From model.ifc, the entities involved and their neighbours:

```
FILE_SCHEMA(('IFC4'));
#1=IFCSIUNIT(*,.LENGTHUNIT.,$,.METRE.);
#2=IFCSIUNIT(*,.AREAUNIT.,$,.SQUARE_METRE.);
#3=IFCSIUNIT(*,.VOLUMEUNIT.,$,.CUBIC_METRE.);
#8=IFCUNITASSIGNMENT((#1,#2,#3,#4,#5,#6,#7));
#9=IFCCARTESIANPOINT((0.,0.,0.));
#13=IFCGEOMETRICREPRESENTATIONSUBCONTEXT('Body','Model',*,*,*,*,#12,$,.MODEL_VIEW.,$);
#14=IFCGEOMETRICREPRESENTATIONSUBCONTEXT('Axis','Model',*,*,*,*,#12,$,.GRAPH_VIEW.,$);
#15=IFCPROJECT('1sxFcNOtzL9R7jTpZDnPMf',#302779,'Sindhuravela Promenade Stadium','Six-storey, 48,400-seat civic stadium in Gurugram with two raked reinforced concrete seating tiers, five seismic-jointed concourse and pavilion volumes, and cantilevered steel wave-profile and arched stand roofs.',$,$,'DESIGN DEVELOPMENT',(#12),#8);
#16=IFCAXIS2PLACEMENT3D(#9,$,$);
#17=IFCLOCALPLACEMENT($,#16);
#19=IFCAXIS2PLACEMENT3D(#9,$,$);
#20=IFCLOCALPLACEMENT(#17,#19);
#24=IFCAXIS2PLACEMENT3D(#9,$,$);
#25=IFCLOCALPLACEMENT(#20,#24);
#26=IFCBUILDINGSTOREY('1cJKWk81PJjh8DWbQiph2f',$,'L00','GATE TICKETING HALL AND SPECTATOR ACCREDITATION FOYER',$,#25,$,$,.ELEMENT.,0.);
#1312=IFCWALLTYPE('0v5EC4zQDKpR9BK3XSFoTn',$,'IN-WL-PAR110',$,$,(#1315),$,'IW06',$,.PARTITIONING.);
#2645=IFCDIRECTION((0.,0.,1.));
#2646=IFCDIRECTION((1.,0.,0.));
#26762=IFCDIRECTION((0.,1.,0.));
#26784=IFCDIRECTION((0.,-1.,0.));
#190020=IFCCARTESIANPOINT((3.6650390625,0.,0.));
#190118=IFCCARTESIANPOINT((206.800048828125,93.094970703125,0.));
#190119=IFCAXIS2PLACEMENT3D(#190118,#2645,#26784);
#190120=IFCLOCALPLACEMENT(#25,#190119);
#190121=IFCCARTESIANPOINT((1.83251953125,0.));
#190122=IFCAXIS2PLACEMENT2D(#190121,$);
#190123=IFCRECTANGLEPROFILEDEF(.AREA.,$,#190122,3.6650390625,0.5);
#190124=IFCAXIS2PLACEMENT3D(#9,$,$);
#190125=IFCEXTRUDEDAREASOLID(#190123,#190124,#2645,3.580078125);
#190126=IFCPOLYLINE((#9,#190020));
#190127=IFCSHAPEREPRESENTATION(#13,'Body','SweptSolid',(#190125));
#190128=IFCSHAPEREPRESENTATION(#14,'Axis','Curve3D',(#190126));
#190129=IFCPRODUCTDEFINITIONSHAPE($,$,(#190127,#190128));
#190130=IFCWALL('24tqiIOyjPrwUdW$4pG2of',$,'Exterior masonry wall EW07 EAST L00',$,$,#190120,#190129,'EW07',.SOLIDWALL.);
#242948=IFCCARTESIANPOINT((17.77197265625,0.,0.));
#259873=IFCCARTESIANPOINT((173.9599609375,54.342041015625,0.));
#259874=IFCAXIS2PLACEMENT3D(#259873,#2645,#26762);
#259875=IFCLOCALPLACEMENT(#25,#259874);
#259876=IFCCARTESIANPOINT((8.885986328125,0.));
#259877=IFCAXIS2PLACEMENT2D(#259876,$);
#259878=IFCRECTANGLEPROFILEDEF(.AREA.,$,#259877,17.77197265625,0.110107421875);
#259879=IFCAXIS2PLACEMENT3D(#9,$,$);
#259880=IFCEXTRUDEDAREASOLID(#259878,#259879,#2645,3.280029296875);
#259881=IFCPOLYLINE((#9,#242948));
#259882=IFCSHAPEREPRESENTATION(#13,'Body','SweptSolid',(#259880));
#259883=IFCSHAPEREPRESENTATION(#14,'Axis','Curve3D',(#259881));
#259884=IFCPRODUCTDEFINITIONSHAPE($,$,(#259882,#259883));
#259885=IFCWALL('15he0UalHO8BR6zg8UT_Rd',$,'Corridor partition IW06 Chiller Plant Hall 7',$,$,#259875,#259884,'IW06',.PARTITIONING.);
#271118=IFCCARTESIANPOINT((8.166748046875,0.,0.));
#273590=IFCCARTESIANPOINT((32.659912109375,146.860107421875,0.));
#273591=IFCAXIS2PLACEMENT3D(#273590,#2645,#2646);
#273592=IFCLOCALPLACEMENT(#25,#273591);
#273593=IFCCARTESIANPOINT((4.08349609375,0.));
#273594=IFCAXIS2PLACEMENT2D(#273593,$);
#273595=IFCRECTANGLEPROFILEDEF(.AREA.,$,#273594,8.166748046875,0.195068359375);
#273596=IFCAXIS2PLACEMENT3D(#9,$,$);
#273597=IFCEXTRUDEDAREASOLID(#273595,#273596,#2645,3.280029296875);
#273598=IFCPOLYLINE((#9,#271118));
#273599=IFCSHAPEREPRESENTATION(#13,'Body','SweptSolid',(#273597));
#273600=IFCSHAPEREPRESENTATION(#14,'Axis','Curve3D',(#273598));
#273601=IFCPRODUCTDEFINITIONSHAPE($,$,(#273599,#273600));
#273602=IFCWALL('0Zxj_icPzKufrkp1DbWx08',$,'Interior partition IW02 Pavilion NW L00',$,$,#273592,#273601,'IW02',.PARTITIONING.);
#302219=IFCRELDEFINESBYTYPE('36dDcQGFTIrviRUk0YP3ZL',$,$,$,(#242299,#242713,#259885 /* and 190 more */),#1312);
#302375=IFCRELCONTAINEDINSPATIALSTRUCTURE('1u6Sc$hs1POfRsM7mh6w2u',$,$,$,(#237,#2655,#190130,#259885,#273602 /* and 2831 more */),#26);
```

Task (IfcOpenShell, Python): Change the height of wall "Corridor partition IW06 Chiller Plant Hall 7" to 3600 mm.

```python
import ifcopenshell
import ifcopenshell.geom
import ifcopenshell.util.representation
import ifcopenshell.util.shape
import ifcopenshell.util.unit

model = ifcopenshell.open("model.ifc")
unit_scale = ifcopenshell.util.unit.calculate_unit_scale(model)
settings = ifcopenshell.geom.settings()


def volume(element):
    """Net volume in cubic metres, openings subtracted."""
    shape = ifcopenshell.geom.create_shape(settings, element)
    return ifcopenshell.util.shape.get_volume(shape.geometry)


wall = model.by_guid("15he0UalHO8BR6zg8UT_Rd")
before = volume(wall)

body = ifcopenshell.util.representation.get_representation(wall, "Model", "Body")
solid = body.Items[0]
old_height = solid.Depth
solid.Depth = 3.6 / unit_scale
after = volume(wall)

print(f"height {old_height:g} -> {solid.Depth:g}, volume {before:.3f} -> {after:.3f} m3")

model.write("model_rev.ifc")
```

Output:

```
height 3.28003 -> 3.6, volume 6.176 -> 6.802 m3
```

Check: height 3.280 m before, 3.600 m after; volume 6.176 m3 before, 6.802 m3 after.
